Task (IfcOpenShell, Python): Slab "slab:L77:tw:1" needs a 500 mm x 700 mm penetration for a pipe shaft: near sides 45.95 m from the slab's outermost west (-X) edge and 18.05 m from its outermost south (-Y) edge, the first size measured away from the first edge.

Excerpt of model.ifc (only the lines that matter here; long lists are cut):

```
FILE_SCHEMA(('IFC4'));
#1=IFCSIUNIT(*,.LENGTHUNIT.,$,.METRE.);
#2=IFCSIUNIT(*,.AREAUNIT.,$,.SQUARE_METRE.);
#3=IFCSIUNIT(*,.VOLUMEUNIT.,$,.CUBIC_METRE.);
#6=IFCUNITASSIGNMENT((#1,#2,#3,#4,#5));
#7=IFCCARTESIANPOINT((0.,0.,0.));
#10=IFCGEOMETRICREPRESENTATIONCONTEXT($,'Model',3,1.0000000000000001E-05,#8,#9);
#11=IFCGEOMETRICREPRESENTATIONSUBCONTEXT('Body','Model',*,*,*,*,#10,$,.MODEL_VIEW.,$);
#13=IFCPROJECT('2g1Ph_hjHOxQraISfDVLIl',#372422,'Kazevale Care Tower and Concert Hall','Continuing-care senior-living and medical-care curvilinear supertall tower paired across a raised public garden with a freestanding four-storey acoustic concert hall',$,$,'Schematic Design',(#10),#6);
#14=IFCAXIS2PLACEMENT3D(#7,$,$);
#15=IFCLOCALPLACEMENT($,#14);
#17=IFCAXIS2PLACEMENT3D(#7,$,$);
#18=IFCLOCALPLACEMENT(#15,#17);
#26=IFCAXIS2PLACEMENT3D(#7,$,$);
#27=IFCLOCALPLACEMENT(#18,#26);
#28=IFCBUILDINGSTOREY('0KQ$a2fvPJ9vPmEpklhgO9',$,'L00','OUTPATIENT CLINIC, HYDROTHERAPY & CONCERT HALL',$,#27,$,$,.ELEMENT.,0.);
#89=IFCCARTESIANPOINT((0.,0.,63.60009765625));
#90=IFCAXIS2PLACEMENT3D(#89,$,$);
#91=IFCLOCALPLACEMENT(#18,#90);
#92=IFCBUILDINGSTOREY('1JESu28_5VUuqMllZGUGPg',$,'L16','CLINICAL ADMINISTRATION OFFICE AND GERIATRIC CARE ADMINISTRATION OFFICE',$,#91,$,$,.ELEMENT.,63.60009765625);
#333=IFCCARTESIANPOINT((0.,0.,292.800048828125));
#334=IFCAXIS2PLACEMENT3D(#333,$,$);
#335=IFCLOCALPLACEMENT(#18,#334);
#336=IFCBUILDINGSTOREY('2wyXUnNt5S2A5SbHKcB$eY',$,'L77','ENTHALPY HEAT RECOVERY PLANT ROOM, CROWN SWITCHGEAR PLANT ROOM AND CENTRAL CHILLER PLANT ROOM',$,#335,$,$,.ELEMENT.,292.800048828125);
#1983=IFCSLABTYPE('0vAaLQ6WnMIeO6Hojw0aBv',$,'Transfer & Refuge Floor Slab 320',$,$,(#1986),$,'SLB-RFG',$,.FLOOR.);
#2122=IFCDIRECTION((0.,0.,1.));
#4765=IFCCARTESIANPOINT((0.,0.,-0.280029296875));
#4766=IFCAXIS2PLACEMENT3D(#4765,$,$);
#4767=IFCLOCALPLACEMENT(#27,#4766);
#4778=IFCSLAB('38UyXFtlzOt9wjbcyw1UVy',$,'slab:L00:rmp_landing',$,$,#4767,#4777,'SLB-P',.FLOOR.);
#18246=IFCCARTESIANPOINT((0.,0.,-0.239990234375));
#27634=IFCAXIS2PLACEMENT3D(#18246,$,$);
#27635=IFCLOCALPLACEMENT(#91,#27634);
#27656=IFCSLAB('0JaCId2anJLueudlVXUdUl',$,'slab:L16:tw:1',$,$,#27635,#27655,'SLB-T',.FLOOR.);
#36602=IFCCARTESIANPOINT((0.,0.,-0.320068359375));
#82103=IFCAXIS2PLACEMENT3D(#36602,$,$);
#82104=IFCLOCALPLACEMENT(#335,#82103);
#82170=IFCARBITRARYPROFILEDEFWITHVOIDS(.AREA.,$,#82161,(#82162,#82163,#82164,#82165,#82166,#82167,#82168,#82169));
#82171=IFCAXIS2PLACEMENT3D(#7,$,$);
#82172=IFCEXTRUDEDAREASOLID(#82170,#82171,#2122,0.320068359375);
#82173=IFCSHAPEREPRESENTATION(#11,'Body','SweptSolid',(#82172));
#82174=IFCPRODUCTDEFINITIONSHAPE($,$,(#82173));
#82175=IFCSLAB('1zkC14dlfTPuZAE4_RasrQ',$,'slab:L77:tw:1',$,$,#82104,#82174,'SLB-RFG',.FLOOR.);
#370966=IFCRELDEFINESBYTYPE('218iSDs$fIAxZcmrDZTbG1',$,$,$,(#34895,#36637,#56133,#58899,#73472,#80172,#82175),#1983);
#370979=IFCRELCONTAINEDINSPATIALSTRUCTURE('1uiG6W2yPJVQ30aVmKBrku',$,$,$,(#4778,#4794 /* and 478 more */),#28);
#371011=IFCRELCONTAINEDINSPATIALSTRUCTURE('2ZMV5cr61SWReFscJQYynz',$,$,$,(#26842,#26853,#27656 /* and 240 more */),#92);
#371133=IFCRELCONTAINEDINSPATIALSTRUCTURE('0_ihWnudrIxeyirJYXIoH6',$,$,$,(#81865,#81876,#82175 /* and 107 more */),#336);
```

```python
import numpy as np
import ifcopenshell
import ifcopenshell.api.feature
import ifcopenshell.api.geometry
import ifcopenshell.api.root
import ifcopenshell.geom
import ifcopenshell.util.placement
import ifcopenshell.util.representation
import ifcopenshell.util.shape
import ifcopenshell.util.unit

model = ifcopenshell.open("model.ifc")
unit_scale = ifcopenshell.util.unit.calculate_unit_scale(model)
settings = ifcopenshell.geom.settings()


def volume(element):
    """Net volume in cubic metres, openings subtracted."""
    shape = ifcopenshell.geom.create_shape(settings, element)
    return ifcopenshell.util.shape.get_volume(shape.geometry)


slab = model.by_guid("1zkC14dlfTPuZAE4_RasrQ")
before = volume(slab)

# Extent in the slab's own axes, in metres. The edges named are its -X and -Y sides.
slab_shape = ifcopenshell.geom.create_shape(settings, slab)
vertices = ifcopenshell.util.shape.get_vertices(slab_shape.geometry)
x_min, y_min, bottom = vertices.min(axis=0)
top = vertices[:, 2].max()

opening = ifcopenshell.api.root.create_entity(model, ifc_class="IfcOpeningElement", name="Pipe shaft opening", predefined_type="OPENING")
context = ifcopenshell.util.representation.get_context(model, "Model", "Body", "MODEL_VIEW")
width, depth = 0.5, 0.7
outline = [(0.0, 0.0), (width, 0.0), (width, depth), (0.0, depth), (0.0, 0.0)]
# Overshoot both faces by 50 mm so the cut is clean.
shape = ifcopenshell.api.geometry.add_slab_representation(
    model, context=context, depth=top - bottom + 0.1, polyline=outline
)
ifcopenshell.api.geometry.assign_representation(model, product=opening, representation=shape)

matrix = ifcopenshell.util.placement.get_local_placement(slab.ObjectPlacement)
matrix[:, 3] = matrix @ np.append(np.array([x_min + 45.95, y_min + 18.05, bottom - 0.05]) / unit_scale, 1.0)
ifcopenshell.api.geometry.edit_object_placement(model, product=opening, matrix=matrix, is_si=False)
ifcopenshell.api.feature.add_feature(model, feature=opening, element=slab)

after = volume(slab)

print(f"slab volume {before:.3f} -> {after:.3f} m3")

model.write("model_edited.ifc")
```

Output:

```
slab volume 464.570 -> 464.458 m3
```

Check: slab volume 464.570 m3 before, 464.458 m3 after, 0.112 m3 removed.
